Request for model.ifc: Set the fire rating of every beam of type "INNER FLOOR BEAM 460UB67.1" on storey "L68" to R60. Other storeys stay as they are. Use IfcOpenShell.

First a look at what the model holds.

```python
import ifcopenshell
import ifcopenshell.util.element

model = ifcopenshell.open("model.ifc")
print(model.schema)
storey = next(s for s in model.by_type("IfcBuildingStorey") if s.Name == "L68")
beams = [e for e in ifcopenshell.util.element.get_decomposition(storey) if e.is_a("IfcBeam")]
seen = {}
for e in beams:
    element_type = ifcopenshell.util.element.get_type(e)
    key = (element_type.Name if element_type != e and element_type else None, ifcopenshell.util.element.get_pset(e, "Pset_BeamCommon", "FireRating"))
    seen[key] = seen.get(key, 0) + 1
for (name, value), count in sorted(seen.items(), key=str):
    print(count, "x", name, "|", value)
```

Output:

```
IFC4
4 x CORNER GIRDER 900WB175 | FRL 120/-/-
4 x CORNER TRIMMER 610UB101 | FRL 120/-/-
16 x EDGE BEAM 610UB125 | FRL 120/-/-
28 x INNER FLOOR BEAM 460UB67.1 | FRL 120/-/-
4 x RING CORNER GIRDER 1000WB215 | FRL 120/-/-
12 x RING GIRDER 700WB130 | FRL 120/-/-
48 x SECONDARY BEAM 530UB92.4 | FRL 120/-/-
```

```python
import ifcopenshell
import ifcopenshell.api.pset
import ifcopenshell.util.element

model = ifcopenshell.open("model.ifc")

storey = next(s for s in model.by_type("IfcBuildingStorey") if s.Name == "L68")
beams = [e for e in ifcopenshell.util.element.get_decomposition(storey) if e.is_a("IfcBeam")]

count = 0
for e in beams:
    element_type = ifcopenshell.util.element.get_type(e)
    if element_type in (None, e) or element_type.Name != "INNER FLOOR BEAM 460UB67.1":
        continue
    found = ifcopenshell.util.element.get_pset(e, "Pset_BeamCommon", should_inherit=False)
    if found:
        pset = model.by_id(found["id"])
        if len(ifcopenshell.util.element.get_elements_by_pset(pset)) > 1:
            pset = ifcopenshell.api.pset.unshare_pset(model, products=[e], pset=pset)[0]
    else:
        pset = ifcopenshell.api.pset.add_pset(model, product=e, name="Pset_BeamCommon")
    ifcopenshell.api.pset.edit_pset(model, pset=pset, properties={"FireRating": "R60"})
    count += 1

print(count, "beams updated")

model.write("model_edited.ifc")
```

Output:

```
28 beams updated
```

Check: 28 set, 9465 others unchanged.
